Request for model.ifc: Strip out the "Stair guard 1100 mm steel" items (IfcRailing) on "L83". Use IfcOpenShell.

First a look at what the model holds.

```python
import ifcopenshell
import ifcopenshell.util.element

model = ifcopenshell.open("model.ifc")
print(model.schema)
storey = next(s for s in model.by_type("IfcBuildingStorey") if s.Name == "L83")
railings = [e for e in ifcopenshell.util.element.get_decomposition(storey) if e.is_a("IfcRailing")]
seen = {}
for e in railings:
    element_type = ifcopenshell.util.element.get_type(e)
    name = element_type.Name if element_type not in (None, e) else None
    seen[name] = seen.get(name, 0) + 1
for name, count in sorted(seen.items(), key=str):
    print(count, "x", name)
```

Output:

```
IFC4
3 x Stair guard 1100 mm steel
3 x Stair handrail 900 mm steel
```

```python
import ifcopenshell
import ifcopenshell.api.root
import ifcopenshell.util.element

model = ifcopenshell.open("model.ifc")

storey = next(s for s in model.by_type("IfcBuildingStorey") if s.Name == "L83")
railings = [e for e in ifcopenshell.util.element.get_decomposition(storey) if e.is_a("IfcRailing")]
targets = [e for e in railings if (t := ifcopenshell.util.element.get_type(e)) not in (None, e) and t.Name == "Stair guard 1100 mm steel"]

for e in targets:
    ifcopenshell.api.root.remove_product(model, product=e)
print(len(targets), "removed")

model.write("model_edited.ifc")
```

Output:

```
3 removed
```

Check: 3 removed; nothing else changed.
